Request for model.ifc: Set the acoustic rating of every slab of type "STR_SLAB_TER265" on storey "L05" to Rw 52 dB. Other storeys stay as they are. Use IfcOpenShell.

First a look at what the model holds.

```python
import ifcopenshell
import ifcopenshell.util.element

model = ifcopenshell.open("model.ifc")
print(model.schema)
storey = next(s for s in model.by_type("IfcBuildingStorey") if s.Name == "L05")
slabs = [e for e in ifcopenshell.util.element.get_decomposition(storey) if e.is_a("IfcSlab")]
seen = {}
for e in slabs:
    element_type = ifcopenshell.util.element.get_type(e)
    key = (element_type.Name if element_type != e and element_type else None, ifcopenshell.util.element.get_pset(e, "Pset_SlabCommon", "AcousticRating"))
    seen[key] = seen.get(key, 0) + 1
for (name, value), count in sorted(seen.items(), key=str):
    print(count, "x", name, "|", value)
```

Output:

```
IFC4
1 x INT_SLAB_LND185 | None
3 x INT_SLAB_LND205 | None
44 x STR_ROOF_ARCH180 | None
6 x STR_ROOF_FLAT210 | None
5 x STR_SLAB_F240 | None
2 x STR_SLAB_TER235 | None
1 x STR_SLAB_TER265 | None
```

```python
import ifcopenshell
import ifcopenshell.api.pset
import ifcopenshell.util.element

model = ifcopenshell.open("model.ifc")

storey = next(s for s in model.by_type("IfcBuildingStorey") if s.Name == "L05")
slabs = [e for e in ifcopenshell.util.element.get_decomposition(storey) if e.is_a("IfcSlab")]

count = 0
for e in slabs:
    element_type = ifcopenshell.util.element.get_type(e)
    if element_type in (None, e) or element_type.Name != "STR_SLAB_TER265":
        continue
    # add_pset returns the element's existing set when there is one.
    pset = ifcopenshell.api.pset.add_pset(model, product=e, name="Pset_SlabCommon")
    ifcopenshell.api.pset.edit_pset(model, pset=pset, properties={"AcousticRating": "Rw 52 dB"})
    count += 1

print(count, "slabs updated")

model.write("model_rev.ifc")
```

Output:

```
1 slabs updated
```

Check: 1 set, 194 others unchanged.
